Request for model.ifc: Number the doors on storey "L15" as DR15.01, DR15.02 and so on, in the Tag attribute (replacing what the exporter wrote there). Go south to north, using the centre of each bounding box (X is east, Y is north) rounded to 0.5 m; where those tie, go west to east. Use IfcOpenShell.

First a look at what the model holds.

```python
import ifcopenshell
import ifcopenshell.util.element
import ifcopenshell.util.placement

model = ifcopenshell.open("model.ifc")
print(model.schema)
storey = next(s for s in model.by_type("IfcBuildingStorey") if s.Name == "L15")
doors = [e for e in ifcopenshell.util.element.get_decomposition(storey) if e.is_a("IfcDoor")]
for e in sorted(doors, key=lambda e: e.id()):
    origin = ifcopenshell.util.placement.get_local_placement(e.ObjectPlacement)[:3, 3]
    print(e.id(), e.Tag, e.Name, origin.round(2) + 0.0, sep=" | ")
```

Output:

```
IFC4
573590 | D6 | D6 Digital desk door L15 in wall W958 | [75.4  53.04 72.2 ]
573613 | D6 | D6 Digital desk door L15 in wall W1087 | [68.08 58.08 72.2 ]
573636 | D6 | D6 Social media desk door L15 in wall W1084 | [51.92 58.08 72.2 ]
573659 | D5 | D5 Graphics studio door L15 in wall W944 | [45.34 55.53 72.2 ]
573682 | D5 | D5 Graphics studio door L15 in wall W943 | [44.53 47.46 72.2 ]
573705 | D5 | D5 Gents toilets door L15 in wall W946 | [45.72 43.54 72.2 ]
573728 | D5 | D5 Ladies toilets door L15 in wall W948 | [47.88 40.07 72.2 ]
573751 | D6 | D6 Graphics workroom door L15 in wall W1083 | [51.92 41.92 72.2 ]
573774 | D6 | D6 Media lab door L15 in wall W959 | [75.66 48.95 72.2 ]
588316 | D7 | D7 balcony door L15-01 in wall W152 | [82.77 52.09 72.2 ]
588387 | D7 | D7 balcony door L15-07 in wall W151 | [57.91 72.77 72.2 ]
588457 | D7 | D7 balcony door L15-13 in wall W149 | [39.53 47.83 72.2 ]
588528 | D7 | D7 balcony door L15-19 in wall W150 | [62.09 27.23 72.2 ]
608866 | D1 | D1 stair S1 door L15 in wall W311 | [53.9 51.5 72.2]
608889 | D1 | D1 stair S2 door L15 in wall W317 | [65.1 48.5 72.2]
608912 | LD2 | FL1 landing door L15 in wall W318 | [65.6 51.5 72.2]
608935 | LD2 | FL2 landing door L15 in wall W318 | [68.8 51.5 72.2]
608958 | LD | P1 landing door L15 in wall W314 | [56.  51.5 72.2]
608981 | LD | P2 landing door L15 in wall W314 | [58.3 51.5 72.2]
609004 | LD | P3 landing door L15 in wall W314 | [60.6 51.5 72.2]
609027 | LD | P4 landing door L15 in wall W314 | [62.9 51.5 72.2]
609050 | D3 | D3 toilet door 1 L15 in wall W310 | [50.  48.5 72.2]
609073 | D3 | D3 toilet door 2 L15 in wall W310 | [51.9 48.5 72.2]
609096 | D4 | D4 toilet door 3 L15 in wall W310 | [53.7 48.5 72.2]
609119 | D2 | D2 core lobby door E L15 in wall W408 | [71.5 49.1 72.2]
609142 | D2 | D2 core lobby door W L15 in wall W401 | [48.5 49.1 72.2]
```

```python
import ifcopenshell
import ifcopenshell.geom
import ifcopenshell.util.element
import ifcopenshell.util.shape

model = ifcopenshell.open("model.ifc")
settings = ifcopenshell.geom.settings()
settings.set("use-world-coords", True)


def centre(element):
    shape = ifcopenshell.geom.create_shape(settings, element)
    return ifcopenshell.util.shape.get_bbox_centroid(shape.geometry)


storey = next(s for s in model.by_type("IfcBuildingStorey") if s.Name == "L15")
doors = [e for e in ifcopenshell.util.element.get_decomposition(storey) if e.is_a("IfcDoor")]

# Insertion points can sit at a corner or the storey origin, so sort by the geometry (in metres).
centres = {e: centre(e) for e in doors}
doors.sort(key=lambda e: (round(centres[e][1] / 0.5), centres[e][0]))

for i, e in enumerate(doors, start=1):
    number = f"DR15.{i:02d}"
    e.Tag = number
    print(e.id(), number)

model.write("model_v2.ifc")
```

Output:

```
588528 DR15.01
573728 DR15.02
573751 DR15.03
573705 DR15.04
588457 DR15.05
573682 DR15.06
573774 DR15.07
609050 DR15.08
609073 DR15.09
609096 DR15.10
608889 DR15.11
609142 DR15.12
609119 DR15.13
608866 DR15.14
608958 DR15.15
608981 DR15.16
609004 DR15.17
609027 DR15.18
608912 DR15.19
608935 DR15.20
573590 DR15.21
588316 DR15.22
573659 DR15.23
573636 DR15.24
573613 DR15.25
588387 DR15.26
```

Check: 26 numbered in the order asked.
